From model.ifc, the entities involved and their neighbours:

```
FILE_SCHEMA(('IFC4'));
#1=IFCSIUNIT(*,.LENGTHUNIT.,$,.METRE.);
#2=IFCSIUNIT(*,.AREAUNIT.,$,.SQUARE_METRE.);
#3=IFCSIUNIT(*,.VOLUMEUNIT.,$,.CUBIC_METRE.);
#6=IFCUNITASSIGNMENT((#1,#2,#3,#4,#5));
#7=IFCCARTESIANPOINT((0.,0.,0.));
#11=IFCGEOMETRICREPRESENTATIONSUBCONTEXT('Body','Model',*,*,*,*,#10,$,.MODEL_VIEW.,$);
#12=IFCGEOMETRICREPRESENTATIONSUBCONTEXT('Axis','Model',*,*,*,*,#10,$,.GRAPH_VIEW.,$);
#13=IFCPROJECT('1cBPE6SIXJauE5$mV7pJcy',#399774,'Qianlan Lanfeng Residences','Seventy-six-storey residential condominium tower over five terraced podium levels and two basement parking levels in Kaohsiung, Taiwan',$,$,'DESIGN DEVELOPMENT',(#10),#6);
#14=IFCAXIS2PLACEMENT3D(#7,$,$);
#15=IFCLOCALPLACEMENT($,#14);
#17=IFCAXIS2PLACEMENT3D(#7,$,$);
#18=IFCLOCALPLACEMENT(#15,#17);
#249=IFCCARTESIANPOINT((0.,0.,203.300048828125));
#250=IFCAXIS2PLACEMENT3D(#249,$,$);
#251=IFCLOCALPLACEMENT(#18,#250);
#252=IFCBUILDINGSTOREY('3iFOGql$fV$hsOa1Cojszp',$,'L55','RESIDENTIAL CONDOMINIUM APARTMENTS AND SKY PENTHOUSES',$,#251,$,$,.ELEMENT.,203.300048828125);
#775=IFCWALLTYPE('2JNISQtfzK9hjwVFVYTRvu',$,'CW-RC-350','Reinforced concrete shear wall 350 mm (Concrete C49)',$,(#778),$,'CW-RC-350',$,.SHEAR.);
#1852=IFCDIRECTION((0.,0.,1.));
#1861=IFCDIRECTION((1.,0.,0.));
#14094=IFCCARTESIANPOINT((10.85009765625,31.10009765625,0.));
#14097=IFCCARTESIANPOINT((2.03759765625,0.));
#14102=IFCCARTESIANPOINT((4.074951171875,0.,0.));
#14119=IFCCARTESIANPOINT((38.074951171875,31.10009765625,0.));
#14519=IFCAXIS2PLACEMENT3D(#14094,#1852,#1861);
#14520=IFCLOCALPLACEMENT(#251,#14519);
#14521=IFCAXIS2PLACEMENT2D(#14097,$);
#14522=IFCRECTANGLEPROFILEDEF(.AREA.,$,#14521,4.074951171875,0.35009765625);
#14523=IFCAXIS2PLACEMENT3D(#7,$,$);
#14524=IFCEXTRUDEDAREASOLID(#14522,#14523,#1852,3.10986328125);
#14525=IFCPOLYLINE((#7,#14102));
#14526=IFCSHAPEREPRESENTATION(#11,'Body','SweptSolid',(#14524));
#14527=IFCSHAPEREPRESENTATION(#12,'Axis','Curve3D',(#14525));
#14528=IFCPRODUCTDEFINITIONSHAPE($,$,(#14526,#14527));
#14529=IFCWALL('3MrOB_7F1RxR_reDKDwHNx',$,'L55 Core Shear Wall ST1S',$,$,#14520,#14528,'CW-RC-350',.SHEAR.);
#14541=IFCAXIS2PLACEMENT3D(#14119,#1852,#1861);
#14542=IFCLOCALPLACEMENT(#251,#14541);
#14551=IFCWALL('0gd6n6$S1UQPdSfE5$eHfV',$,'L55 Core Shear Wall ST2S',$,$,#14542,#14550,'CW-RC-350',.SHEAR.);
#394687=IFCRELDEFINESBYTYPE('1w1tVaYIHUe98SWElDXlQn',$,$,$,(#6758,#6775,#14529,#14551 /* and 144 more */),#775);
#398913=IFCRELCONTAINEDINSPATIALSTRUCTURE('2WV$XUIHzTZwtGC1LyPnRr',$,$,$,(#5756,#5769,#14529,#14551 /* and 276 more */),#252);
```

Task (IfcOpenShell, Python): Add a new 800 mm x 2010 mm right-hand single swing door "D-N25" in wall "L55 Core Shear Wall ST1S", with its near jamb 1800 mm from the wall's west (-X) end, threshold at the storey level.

```python
import numpy as np
import ifcopenshell
import ifcopenshell.api.feature
import ifcopenshell.api.geometry
import ifcopenshell.api.root
import ifcopenshell.api.spatial
import ifcopenshell.geom
import ifcopenshell.util.element
import ifcopenshell.util.placement
import ifcopenshell.util.representation
import ifcopenshell.util.shape
import ifcopenshell.util.unit

model = ifcopenshell.open("model.ifc")
unit_scale = ifcopenshell.util.unit.calculate_unit_scale(model)
settings = ifcopenshell.geom.settings()


def volume(element):
    """Net volume in cubic metres, openings subtracted."""
    shape = ifcopenshell.geom.create_shape(settings, element)
    return ifcopenshell.util.shape.get_volume(shape.geometry)


wall = model.by_guid("3MrOB_7F1RxR_reDKDwHNx")
storey = ifcopenshell.util.element.get_container(wall, ifc_class="IfcBuildingStorey")
context = ifcopenshell.util.representation.get_context(model, "Model", "Body", "MODEL_VIEW")
before = volume(wall)

width, height, from_end, sill = 0.8, 2.01, 1.8, 0.0  # metres

# The wall runs along its own X axis, and the end named is its -X end.
wall_shape = ifcopenshell.geom.create_shape(settings, wall)
x, y, z = ifcopenshell.util.shape.get_vertices(wall_shape.geometry).T
start = x.min() + from_end
face, thickness = float(y.min()), float(y.max() - y.min())
wall_matrix = ifcopenshell.util.placement.get_local_placement(wall.ObjectPlacement)
level = ifcopenshell.util.placement.get_local_placement(storey.ObjectPlacement)[2, 3]


def in_wall(x, y):
    """Placement at x, y metres in the wall's axes, at sill height."""
    matrix = wall_matrix.copy()
    matrix[:, 3] = wall_matrix @ np.array([x / unit_scale, y / unit_scale, 0.0, 1.0])
    matrix[2, 3] = level + sill / unit_scale
    return matrix


# Opening: a box that overshoots both wall faces by 50 mm.
opening = ifcopenshell.api.root.create_entity(model, ifc_class="IfcOpeningElement", predefined_type="OPENING")
box = ifcopenshell.api.geometry.add_wall_representation(
    model, context=context, length=width, height=height, thickness=thickness + 0.1
)
ifcopenshell.api.geometry.assign_representation(model, product=opening, representation=box)
ifcopenshell.api.geometry.edit_object_placement(model, product=opening, matrix=in_wall(start, face - 0.05), is_si=False)
ifcopenshell.api.feature.add_feature(model, feature=opening, element=wall)

door = ifcopenshell.api.root.create_entity(model, ifc_class="IfcDoor", name="D-N25", predefined_type="DOOR")
door.OverallWidth, door.OverallHeight = width / unit_scale, height / unit_scale
door.OperationType = "SINGLE_SWING_RIGHT"
body = ifcopenshell.api.geometry.add_door_representation(
    model,
    context=context,
    overall_width=door.OverallWidth,
    overall_height=door.OverallHeight,
    operation_type="SINGLE_SWING_RIGHT",
    lining_properties={"LiningDepth": thickness / unit_scale, "ThresholdDepth": thickness / unit_scale},
)
ifcopenshell.api.geometry.assign_representation(model, product=door, representation=body)
ifcopenshell.api.spatial.assign_container(model, products=[door], relating_structure=storey)
ifcopenshell.api.feature.add_filling(model, opening=opening, element=door)

# The lining spans the wall, so the door starts at the wall face.
ifcopenshell.api.geometry.edit_object_placement(model, product=door, matrix=in_wall(start, face), is_si=False)

after = volume(wall)

print(f"wall volume {before:.3f} -> {after:.3f} m3")

model.write("model_rev.ifc")
```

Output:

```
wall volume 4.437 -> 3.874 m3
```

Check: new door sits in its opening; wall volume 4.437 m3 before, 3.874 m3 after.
